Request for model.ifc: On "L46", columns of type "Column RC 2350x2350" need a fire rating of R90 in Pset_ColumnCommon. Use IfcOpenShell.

First a look at what the model holds.

```python
import ifcopenshell
import ifcopenshell.util.element

model = ifcopenshell.open("model.ifc")
print(model.schema)
storey = next(s for s in model.by_type("IfcBuildingStorey") if s.Name == "L46")
columns = [e for e in ifcopenshell.util.element.get_decomposition(storey) if e.is_a("IfcColumn")]
seen = {}
for e in columns:
    element_type = ifcopenshell.util.element.get_type(e)
    key = (element_type.Name if element_type != e and element_type else None, ifcopenshell.util.element.get_pset(e, "Pset_ColumnCommon", "FireRating"))
    seen[key] = seen.get(key, 0) + 1
for (name, value), count in sorted(seen.items(), key=str):
    print(count, "x", name, "|", value)
```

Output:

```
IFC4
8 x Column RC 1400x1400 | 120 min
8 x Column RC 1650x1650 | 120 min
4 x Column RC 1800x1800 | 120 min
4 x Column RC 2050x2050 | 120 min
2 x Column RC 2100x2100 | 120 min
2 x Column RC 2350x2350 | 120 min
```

```python
import ifcopenshell
import ifcopenshell.api.pset
import ifcopenshell.util.element

model = ifcopenshell.open("model.ifc")

storey = next(s for s in model.by_type("IfcBuildingStorey") if s.Name == "L46")
columns = [e for e in ifcopenshell.util.element.get_decomposition(storey) if e.is_a("IfcColumn")]

count = 0
for e in columns:
    element_type = ifcopenshell.util.element.get_type(e)
    if element_type in (None, e) or element_type.Name != "Column RC 2350x2350":
        continue
    # add_pset returns the element's existing set when there is one.
    pset = ifcopenshell.api.pset.add_pset(model, product=e, name="Pset_ColumnCommon")
    ifcopenshell.api.pset.edit_pset(model, pset=pset, properties={"FireRating": "R90"})
    count += 1

print(count, "columns updated")

model.write("model_edited.ifc")
```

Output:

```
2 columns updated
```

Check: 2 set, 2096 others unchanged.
